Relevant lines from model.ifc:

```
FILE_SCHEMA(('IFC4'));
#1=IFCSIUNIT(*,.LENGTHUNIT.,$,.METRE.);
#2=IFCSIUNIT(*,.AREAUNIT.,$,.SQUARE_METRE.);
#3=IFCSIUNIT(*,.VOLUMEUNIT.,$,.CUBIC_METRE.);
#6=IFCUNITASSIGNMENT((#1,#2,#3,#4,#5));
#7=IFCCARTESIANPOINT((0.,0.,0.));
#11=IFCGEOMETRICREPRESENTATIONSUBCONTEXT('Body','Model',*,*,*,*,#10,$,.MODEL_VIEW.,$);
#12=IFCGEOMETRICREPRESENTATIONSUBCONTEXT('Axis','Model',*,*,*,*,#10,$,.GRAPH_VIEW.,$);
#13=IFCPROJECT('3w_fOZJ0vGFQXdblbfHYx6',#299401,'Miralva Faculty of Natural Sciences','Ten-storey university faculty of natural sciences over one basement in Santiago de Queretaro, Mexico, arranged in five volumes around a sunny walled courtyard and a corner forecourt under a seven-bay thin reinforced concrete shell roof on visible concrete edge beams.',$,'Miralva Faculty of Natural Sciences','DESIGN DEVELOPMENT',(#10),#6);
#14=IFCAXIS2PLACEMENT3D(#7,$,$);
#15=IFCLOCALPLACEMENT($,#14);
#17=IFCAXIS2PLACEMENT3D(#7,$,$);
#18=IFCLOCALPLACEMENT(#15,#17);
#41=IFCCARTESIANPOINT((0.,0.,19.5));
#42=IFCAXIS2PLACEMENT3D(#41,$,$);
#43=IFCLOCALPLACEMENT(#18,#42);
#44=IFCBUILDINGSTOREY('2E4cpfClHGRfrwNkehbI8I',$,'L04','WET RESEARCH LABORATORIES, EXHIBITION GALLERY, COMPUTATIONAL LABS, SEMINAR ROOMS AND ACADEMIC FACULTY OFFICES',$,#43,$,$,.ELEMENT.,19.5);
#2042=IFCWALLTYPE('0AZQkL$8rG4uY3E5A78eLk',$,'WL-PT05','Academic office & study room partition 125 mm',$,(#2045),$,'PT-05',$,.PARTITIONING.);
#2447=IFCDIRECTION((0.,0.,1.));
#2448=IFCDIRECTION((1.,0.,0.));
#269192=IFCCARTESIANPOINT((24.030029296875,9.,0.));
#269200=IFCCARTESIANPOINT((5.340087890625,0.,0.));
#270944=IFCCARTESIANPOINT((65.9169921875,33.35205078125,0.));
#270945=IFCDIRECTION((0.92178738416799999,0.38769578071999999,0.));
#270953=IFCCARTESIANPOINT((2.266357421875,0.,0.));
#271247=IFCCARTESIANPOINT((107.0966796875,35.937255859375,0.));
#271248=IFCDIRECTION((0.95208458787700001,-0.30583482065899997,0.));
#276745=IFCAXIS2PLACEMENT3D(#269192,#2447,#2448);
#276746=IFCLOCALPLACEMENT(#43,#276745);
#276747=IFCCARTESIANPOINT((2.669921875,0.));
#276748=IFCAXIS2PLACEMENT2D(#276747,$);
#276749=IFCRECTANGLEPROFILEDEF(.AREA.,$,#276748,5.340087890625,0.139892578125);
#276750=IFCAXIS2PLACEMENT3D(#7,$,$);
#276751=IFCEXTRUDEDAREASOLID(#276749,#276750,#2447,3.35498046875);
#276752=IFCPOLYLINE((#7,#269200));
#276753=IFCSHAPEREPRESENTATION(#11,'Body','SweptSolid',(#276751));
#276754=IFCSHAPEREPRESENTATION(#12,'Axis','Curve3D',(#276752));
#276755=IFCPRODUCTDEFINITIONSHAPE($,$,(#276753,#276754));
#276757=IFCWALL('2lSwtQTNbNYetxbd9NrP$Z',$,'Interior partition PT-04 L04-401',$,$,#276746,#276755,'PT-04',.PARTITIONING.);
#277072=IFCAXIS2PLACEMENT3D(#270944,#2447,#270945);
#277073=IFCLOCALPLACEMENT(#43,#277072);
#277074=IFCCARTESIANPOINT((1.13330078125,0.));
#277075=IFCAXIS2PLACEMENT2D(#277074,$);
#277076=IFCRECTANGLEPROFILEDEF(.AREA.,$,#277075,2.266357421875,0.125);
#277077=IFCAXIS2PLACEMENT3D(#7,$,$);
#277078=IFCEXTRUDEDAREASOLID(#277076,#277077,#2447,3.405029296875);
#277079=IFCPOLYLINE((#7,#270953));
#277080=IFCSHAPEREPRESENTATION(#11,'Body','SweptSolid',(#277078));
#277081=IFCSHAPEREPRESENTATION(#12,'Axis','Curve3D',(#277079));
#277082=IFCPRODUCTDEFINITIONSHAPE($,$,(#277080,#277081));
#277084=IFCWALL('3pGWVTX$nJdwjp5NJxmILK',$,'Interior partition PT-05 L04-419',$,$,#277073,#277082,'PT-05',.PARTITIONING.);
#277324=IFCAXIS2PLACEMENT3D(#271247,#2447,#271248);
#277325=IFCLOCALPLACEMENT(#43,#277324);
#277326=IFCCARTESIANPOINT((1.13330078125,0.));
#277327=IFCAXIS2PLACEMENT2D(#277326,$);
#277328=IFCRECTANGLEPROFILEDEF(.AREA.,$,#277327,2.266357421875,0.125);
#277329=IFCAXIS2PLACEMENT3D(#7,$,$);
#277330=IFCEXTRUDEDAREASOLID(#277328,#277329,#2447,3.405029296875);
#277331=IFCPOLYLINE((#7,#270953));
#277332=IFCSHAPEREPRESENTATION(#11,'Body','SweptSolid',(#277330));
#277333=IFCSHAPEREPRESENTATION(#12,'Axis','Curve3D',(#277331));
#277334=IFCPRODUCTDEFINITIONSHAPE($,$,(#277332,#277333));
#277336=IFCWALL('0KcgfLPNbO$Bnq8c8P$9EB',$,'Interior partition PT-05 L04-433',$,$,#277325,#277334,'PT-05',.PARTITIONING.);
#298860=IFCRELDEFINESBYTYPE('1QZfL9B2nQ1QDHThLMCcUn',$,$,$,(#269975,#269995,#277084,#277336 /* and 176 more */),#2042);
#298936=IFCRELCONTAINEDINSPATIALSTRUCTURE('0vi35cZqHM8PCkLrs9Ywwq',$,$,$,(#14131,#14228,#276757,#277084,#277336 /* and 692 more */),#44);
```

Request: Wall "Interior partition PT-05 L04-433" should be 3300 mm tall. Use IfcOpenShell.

```python
import ifcopenshell
import ifcopenshell.geom
import ifcopenshell.util.representation
import ifcopenshell.util.shape

model = ifcopenshell.open("model.ifc")
settings = ifcopenshell.geom.settings()


def volume(element):
    """Net volume in cubic metres, openings subtracted."""
    shape = ifcopenshell.geom.create_shape(settings, element)
    return ifcopenshell.util.shape.get_volume(shape.geometry)


wall = model.by_guid("0KcgfLPNbO$Bnq8c8P$9EB")
before = volume(wall)

body = ifcopenshell.util.representation.get_representation(wall, "Model", "Body")
solid = body.Items[0]
old_height = solid.Depth
solid.Depth = 3.3
after = volume(wall)

print(f"height {old_height:g} -> {solid.Depth:g}, volume {before:.3f} -> {after:.3f} m3")

model.write("model_rev.ifc")
```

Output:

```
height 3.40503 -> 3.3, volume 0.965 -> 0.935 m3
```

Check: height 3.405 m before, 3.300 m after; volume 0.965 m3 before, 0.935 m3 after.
